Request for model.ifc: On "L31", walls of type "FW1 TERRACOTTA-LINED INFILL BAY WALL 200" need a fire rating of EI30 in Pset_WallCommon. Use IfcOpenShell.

First a look at what the model holds.

```python
import ifcopenshell
import ifcopenshell.util.element

model = ifcopenshell.open("model.ifc")
print(model.schema)
storey = next(s for s in model.by_type("IfcBuildingStorey") if s.Name == "L31")
walls = [e for e in ifcopenshell.util.element.get_decomposition(storey) if e.is_a("IfcWall")]
seen = {}
for e in walls:
    element_type = ifcopenshell.util.element.get_type(e)
    key = (element_type.Name if element_type != e and element_type else None, ifcopenshell.util.element.get_pset(e, "Pset_WallCommon", "FireRating"))
    seen[key] = seen.get(key, 0) + 1
for (name, value), count in sorted(seen.items(), key=str):
    print(count, "x", name, "|", value)
```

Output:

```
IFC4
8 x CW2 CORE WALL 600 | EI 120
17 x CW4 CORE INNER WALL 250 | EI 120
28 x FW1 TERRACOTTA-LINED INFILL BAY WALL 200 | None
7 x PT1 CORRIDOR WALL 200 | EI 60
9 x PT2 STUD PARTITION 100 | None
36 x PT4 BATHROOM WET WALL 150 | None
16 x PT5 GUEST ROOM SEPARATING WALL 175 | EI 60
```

```python
import ifcopenshell
import ifcopenshell.api.pset
import ifcopenshell.util.element

model = ifcopenshell.open("model.ifc")

storey = next(s for s in model.by_type("IfcBuildingStorey") if s.Name == "L31")
walls = [e for e in ifcopenshell.util.element.get_decomposition(storey) if e.is_a("IfcWall")]

count = 0
for e in walls:
    element_type = ifcopenshell.util.element.get_type(e)
    if element_type in (None, e) or element_type.Name != "FW1 TERRACOTTA-LINED INFILL BAY WALL 200":
        continue
    found = ifcopenshell.util.element.get_pset(e, "Pset_WallCommon", should_inherit=False)
    if found:
        pset = model.by_id(found["id"])
        if len(ifcopenshell.util.element.get_elements_by_pset(pset)) > 1:
            pset = ifcopenshell.api.pset.unshare_pset(model, products=[e], pset=pset)[0]
    else:
        pset = ifcopenshell.api.pset.add_pset(model, product=e, name="Pset_WallCommon")
    ifcopenshell.api.pset.edit_pset(model, pset=pset, properties={"FireRating": "EI30"})
    count += 1

print(count, "walls updated")

model.write("model_v2.ifc")
```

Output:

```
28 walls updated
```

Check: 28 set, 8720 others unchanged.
